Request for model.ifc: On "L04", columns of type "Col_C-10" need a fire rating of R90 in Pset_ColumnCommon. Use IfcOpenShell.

First a look at what the model holds.

```python
import ifcopenshell
import ifcopenshell.util.element

model = ifcopenshell.open("model.ifc")
print(model.schema)
storey = next(s for s in model.by_type("IfcBuildingStorey") if s.Name == "L04")
columns = [e for e in ifcopenshell.util.element.get_decomposition(storey) if e.is_a("IfcColumn")]
seen = {}
for e in columns:
    element_type = ifcopenshell.util.element.get_type(e)
    key = (element_type.Name if element_type != e and element_type else None, ifcopenshell.util.element.get_pset(e, "Pset_ColumnCommon", "FireRating"))
    seen[key] = seen.get(key, 0) + 1
for (name, value), count in sorted(seen.items(), key=str):
    print(count, "x", name, "|", value)
```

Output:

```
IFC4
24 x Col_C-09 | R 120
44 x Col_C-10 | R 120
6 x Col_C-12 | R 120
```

```python
import ifcopenshell
import ifcopenshell.api.pset
import ifcopenshell.util.element

model = ifcopenshell.open("model.ifc")

storey = next(s for s in model.by_type("IfcBuildingStorey") if s.Name == "L04")
columns = [e for e in ifcopenshell.util.element.get_decomposition(storey) if e.is_a("IfcColumn")]

count = 0
for e in columns:
    element_type = ifcopenshell.util.element.get_type(e)
    if element_type in (None, e) or element_type.Name != "Col_C-10":
        continue
    # add_pset returns the element's existing set when there is one.
    pset = ifcopenshell.api.pset.add_pset(model, product=e, name="Pset_ColumnCommon")
    ifcopenshell.api.pset.edit_pset(model, pset=pset, properties={"FireRating": "R90"})
    count += 1

print(count, "columns updated")

model.write("model-out.ifc")
```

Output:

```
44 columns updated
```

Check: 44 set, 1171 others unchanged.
